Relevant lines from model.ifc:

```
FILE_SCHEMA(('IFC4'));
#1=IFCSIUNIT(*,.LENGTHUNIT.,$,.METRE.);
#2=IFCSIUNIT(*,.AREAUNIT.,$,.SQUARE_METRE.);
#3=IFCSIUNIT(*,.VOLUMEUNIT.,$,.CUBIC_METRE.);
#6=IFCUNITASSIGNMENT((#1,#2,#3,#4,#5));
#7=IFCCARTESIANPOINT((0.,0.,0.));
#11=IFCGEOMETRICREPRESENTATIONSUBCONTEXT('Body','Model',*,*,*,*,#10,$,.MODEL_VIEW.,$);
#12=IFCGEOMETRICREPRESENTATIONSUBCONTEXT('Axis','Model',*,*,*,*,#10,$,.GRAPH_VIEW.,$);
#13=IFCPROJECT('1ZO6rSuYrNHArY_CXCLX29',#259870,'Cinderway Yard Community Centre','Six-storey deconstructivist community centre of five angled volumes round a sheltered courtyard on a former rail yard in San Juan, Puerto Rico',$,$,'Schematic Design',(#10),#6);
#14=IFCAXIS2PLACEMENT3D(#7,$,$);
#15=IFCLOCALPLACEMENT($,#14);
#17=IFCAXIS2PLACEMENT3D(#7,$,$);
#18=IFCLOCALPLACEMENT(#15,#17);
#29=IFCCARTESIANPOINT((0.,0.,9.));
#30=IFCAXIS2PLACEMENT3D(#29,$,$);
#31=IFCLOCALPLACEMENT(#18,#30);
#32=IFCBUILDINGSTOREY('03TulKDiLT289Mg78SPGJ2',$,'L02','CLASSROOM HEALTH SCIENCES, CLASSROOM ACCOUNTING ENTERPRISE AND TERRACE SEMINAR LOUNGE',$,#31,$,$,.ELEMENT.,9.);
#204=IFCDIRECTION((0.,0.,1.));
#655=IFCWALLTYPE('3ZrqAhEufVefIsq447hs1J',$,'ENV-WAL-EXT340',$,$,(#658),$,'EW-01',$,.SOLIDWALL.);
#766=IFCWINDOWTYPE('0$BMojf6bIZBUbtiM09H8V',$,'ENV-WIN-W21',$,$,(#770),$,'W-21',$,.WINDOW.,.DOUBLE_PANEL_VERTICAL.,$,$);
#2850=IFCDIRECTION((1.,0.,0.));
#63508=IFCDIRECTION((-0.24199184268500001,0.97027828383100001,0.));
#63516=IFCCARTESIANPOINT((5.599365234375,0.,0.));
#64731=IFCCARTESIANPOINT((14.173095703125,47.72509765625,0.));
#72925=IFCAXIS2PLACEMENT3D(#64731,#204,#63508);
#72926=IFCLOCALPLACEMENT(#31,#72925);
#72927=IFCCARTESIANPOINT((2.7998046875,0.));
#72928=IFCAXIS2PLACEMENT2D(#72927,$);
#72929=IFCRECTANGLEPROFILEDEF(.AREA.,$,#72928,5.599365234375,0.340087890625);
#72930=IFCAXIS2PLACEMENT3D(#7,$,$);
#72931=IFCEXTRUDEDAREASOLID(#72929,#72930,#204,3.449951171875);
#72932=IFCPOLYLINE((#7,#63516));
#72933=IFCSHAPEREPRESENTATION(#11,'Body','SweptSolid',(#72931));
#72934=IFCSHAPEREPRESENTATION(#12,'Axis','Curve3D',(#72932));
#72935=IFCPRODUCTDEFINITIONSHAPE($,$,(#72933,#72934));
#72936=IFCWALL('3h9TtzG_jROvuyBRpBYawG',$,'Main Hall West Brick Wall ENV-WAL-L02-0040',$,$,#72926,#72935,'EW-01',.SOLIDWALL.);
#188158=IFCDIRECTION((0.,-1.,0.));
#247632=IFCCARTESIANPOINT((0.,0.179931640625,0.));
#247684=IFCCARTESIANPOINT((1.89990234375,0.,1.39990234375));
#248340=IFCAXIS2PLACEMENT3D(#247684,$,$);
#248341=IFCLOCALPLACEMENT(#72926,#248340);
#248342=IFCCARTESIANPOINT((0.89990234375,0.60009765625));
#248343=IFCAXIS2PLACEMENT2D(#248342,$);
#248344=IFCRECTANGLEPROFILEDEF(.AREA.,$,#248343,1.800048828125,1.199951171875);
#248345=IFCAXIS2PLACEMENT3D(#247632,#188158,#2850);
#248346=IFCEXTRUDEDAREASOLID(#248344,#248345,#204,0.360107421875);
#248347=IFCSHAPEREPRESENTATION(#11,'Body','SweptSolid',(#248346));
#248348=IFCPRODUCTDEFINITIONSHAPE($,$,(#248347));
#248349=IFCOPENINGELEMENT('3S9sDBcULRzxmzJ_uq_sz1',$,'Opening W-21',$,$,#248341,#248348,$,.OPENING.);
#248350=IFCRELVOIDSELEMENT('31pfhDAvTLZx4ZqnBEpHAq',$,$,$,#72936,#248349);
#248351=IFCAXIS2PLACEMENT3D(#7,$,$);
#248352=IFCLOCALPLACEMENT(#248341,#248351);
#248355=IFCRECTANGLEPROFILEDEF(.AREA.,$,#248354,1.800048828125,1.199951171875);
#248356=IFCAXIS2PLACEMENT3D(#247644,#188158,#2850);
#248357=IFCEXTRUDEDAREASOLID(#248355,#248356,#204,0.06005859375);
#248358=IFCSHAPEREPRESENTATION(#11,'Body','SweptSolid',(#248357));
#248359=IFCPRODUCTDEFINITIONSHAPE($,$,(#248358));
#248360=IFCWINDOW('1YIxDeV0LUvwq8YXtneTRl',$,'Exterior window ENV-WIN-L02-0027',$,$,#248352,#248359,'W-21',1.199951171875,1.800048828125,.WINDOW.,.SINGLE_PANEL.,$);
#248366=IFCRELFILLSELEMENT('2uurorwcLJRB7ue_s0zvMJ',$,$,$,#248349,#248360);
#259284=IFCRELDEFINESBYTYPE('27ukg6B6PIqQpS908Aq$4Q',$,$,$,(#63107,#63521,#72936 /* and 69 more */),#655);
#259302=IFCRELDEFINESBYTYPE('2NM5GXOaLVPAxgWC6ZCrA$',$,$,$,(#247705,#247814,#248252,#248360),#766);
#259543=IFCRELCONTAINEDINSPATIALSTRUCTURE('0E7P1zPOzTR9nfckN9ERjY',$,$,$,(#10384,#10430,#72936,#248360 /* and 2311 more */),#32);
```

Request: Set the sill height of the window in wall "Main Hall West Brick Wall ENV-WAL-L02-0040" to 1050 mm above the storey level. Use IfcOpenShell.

```python
import numpy as np
import ifcopenshell
import ifcopenshell.api.geometry
import ifcopenshell.geom
import ifcopenshell.util.element
import ifcopenshell.util.placement
import ifcopenshell.util.shape
import ifcopenshell.util.unit

model = ifcopenshell.open("model.ifc")
unit_scale = ifcopenshell.util.unit.calculate_unit_scale(model)

window = model.by_guid("1YIxDeV0LUvwq8YXtneTRl")
opening = window.FillsVoids[0].RelatingOpeningElement
storey = ifcopenshell.util.element.get_container(window, ifc_class="IfcBuildingStorey")
level = ifcopenshell.util.placement.get_local_placement(storey.ObjectPlacement)[2, 3]

# The opening's origin need not be at the sill, so measure its lowest point.
shape = ifcopenshell.geom.create_shape(ifcopenshell.geom.settings(), opening)
bottom = ifcopenshell.util.shape.get_shape_bottom_elevation(shape, shape.geometry) / unit_scale
dz = level + 1.05 / unit_scale - bottom

shift = np.array([0.0, 0.0, dz])
# The window is placed relative to its opening, so it follows when the opening moves.
matrix = ifcopenshell.util.placement.get_local_placement(opening.ObjectPlacement)
matrix[:3, 3] += shift
ifcopenshell.api.geometry.edit_object_placement(
    model, product=opening, matrix=matrix, is_si=False, should_transform_children=True
)

print(f"moved by {dz * unit_scale:+.3f} m")

model.write("model_edited.ifc")
```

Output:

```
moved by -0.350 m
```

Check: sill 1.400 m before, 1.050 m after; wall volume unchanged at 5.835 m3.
